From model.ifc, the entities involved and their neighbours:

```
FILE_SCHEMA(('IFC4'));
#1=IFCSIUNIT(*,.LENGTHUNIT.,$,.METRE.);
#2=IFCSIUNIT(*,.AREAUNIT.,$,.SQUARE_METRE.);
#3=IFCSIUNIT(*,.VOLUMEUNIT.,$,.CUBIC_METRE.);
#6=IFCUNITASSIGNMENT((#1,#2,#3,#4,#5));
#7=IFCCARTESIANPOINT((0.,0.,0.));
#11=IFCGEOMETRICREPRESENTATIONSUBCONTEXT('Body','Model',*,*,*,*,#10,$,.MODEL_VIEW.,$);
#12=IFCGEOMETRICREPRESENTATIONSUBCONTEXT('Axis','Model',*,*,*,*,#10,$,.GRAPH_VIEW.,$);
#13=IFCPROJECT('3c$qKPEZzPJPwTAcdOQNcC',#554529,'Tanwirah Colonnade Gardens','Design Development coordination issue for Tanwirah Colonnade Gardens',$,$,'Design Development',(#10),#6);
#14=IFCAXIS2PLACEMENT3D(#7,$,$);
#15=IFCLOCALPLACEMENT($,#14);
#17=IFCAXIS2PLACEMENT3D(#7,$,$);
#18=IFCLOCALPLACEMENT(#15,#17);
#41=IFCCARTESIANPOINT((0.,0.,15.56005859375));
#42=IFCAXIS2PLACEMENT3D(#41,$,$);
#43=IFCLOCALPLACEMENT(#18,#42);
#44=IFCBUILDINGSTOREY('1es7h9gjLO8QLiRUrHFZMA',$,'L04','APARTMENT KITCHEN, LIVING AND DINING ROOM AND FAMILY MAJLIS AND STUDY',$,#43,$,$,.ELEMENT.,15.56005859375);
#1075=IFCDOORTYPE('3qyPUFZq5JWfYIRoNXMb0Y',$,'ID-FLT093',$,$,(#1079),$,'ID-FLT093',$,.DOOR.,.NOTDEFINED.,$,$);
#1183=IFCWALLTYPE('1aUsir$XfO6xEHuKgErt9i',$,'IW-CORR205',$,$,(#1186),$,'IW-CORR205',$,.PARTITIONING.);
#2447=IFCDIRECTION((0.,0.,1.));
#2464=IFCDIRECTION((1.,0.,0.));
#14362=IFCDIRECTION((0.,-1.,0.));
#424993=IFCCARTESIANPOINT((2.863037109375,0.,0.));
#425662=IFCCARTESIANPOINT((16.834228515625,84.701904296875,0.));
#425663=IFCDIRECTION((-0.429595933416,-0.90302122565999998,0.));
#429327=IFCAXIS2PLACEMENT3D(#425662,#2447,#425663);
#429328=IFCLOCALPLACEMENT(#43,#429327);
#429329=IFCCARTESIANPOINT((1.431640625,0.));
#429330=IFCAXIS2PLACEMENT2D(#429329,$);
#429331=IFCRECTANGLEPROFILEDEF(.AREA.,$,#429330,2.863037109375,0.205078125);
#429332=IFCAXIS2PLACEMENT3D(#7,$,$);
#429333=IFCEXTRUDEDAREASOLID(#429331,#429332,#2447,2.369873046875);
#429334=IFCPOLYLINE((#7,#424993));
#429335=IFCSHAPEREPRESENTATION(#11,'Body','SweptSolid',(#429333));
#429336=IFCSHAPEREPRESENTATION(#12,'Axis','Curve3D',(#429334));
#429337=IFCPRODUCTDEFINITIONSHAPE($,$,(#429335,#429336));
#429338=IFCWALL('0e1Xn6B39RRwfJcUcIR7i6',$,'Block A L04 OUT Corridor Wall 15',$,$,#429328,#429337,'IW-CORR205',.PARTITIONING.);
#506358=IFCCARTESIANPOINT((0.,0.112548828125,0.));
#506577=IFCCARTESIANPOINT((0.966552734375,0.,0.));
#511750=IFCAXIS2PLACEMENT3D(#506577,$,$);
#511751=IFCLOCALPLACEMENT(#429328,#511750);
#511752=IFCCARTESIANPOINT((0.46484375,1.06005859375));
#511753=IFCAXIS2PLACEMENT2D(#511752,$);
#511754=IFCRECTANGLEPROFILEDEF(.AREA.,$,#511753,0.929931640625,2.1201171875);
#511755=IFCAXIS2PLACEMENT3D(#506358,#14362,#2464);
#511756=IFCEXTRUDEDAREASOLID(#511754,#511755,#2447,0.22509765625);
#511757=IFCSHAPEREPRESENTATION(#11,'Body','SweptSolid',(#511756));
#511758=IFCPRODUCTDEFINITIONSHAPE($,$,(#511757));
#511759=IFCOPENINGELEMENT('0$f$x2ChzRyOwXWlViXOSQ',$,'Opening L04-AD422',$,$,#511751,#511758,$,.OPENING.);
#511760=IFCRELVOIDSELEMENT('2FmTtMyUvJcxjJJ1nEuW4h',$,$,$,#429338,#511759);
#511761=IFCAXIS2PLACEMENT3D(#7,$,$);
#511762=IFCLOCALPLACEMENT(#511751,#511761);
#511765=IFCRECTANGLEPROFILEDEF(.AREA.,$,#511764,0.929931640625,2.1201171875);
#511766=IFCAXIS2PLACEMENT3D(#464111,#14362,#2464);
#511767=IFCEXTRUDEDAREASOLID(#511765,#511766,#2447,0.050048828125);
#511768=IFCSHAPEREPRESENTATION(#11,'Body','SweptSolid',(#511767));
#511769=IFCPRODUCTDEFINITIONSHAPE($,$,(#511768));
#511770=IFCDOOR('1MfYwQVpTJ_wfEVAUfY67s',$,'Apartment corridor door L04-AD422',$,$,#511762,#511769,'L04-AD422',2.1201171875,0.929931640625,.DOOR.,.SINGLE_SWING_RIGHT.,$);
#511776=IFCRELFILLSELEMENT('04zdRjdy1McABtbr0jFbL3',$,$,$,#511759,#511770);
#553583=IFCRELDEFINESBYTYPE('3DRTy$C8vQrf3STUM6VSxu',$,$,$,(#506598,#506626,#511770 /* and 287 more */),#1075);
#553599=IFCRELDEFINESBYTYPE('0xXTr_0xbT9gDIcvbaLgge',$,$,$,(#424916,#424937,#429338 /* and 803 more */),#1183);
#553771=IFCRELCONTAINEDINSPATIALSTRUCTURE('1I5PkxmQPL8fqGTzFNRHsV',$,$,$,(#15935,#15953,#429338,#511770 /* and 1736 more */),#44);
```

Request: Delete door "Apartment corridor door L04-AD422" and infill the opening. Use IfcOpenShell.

```python
import ifcopenshell
import ifcopenshell.api.feature
import ifcopenshell.api.root
import ifcopenshell.geom
import ifcopenshell.util.shape

model = ifcopenshell.open("model.ifc")
settings = ifcopenshell.geom.settings()


def volume(element):
    """Net volume in cubic metres, openings subtracted."""
    shape = ifcopenshell.geom.create_shape(settings, element)
    return ifcopenshell.util.shape.get_volume(shape.geometry)


door = model.by_guid("1MfYwQVpTJ_wfEVAUfY67s")
opening = door.FillsVoids[0].RelatingOpeningElement
wall = opening.VoidsElements[0].RelatingBuildingElement
before = volume(wall)

ifcopenshell.api.root.remove_product(model, product=door)
ifcopenshell.api.feature.remove_feature(model, feature=opening)

after = volume(wall)

print(f"wall volume {before:.3f} -> {after:.3f} m3")

model.write("model_rev.ifc")
```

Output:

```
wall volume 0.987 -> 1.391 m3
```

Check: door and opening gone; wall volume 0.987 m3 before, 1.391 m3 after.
